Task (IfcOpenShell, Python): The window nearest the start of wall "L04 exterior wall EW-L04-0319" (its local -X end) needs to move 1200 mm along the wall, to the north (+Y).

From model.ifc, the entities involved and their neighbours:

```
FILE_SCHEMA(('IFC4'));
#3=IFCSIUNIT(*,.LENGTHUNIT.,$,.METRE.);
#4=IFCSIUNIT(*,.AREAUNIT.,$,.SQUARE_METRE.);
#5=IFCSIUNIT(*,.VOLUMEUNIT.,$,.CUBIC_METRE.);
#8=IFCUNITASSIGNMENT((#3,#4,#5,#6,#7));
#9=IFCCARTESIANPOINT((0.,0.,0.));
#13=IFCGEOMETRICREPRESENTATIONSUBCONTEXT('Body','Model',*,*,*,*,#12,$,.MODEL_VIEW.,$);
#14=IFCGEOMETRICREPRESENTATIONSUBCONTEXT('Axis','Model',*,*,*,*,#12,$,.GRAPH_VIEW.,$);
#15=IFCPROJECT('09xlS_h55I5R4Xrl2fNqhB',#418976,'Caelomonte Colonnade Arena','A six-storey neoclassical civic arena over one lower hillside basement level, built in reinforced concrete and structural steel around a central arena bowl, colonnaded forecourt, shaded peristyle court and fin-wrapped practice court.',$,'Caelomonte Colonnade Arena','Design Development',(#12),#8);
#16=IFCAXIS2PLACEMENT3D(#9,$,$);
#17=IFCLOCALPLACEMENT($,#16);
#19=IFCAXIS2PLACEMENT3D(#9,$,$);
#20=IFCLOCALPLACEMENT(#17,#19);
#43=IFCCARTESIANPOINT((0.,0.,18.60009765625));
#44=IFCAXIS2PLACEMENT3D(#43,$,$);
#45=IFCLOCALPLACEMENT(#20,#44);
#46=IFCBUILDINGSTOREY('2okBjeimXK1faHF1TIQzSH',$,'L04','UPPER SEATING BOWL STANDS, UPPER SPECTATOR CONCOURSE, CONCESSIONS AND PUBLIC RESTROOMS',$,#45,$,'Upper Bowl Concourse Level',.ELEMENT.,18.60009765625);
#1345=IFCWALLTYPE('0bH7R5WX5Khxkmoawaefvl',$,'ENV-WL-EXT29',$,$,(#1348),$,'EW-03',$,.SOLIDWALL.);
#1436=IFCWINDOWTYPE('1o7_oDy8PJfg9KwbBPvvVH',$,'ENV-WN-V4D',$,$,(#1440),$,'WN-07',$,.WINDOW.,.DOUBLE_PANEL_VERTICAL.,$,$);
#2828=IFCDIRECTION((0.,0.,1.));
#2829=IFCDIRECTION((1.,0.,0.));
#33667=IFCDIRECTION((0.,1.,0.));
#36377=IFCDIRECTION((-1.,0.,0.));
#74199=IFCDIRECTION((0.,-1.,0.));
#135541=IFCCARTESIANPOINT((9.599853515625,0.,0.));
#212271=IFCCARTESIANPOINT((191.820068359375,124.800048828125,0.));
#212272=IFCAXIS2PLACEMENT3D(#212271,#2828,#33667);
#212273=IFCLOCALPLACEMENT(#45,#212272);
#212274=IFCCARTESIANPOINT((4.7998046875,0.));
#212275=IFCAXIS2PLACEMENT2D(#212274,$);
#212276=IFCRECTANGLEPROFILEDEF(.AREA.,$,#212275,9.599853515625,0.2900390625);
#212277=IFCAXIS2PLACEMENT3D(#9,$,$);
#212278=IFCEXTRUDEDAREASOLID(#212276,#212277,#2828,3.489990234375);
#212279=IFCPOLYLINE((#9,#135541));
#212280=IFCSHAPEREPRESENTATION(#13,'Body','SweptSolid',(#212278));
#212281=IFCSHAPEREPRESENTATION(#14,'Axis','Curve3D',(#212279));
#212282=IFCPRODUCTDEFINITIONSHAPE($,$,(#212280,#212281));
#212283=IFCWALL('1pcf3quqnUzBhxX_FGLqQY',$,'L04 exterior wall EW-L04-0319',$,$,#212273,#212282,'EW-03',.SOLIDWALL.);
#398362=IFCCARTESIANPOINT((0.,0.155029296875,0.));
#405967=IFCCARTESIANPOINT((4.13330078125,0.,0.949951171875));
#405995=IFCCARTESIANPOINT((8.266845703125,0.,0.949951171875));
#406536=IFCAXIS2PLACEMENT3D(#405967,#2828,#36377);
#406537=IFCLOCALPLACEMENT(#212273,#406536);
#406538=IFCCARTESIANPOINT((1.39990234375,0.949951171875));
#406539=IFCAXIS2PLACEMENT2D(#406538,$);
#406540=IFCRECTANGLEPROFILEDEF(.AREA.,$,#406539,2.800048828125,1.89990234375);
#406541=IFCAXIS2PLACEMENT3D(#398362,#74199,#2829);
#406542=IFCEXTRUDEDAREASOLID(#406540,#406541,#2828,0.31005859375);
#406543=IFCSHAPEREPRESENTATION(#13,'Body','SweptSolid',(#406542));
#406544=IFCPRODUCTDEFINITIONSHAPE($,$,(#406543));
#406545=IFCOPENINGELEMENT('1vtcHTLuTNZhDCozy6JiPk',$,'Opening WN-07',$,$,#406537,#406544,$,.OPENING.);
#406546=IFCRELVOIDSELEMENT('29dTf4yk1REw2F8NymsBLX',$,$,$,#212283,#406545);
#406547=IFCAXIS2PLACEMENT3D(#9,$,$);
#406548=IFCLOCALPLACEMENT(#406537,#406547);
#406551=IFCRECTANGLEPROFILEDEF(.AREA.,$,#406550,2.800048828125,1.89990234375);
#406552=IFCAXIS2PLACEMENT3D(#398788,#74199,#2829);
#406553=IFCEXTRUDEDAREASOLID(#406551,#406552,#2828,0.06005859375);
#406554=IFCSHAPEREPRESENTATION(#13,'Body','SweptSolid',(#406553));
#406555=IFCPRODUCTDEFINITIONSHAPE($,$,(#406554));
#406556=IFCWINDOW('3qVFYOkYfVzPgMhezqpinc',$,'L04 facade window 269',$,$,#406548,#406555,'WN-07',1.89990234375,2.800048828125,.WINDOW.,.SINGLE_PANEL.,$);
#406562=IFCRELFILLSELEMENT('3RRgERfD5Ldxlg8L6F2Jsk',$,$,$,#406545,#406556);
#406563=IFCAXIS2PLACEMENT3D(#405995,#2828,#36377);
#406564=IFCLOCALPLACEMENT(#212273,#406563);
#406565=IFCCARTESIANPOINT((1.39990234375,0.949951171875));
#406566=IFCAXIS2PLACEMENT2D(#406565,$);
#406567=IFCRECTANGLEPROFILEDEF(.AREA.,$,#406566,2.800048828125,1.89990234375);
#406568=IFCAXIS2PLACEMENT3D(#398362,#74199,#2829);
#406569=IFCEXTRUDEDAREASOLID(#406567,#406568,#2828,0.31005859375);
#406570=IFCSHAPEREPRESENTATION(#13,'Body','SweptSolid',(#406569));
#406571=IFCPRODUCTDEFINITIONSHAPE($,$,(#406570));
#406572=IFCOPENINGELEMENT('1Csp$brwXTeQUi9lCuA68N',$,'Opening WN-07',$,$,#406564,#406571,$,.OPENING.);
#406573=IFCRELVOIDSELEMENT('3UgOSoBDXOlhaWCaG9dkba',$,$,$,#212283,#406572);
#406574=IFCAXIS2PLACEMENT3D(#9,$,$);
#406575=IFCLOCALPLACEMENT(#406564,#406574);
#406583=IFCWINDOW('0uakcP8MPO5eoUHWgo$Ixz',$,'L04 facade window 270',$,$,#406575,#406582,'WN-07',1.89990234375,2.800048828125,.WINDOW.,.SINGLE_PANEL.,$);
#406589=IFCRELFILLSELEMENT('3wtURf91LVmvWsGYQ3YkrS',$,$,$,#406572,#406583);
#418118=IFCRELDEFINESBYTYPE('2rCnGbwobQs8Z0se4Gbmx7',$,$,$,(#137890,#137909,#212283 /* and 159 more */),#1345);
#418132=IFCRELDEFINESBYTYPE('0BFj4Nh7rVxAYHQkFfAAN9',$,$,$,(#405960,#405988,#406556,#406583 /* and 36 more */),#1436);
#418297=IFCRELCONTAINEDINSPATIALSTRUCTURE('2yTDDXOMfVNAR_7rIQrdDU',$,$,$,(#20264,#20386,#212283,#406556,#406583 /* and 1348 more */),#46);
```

```python
import ifcopenshell
import ifcopenshell.api.geometry
import ifcopenshell.util.placement
import ifcopenshell.util.unit

model = ifcopenshell.open("model.ifc")
unit_scale = ifcopenshell.util.unit.calculate_unit_scale(model)

window = model.by_guid("3qVFYOkYfVzPgMhezqpinc")
opening = window.FillsVoids[0].RelatingOpeningElement
wall = opening.VoidsElements[0].RelatingBuildingElement

wall_matrix = ifcopenshell.util.placement.get_local_placement(wall.ObjectPlacement)
shift = wall_matrix[:3, 0] * 1.2 / unit_scale
before = ifcopenshell.util.placement.get_local_placement(window.ObjectPlacement)[:3, 3].copy()

# The window is placed relative to its opening, so it follows when the opening moves.
matrix = ifcopenshell.util.placement.get_local_placement(opening.ObjectPlacement)
matrix[:3, 3] += shift
ifcopenshell.api.geometry.edit_object_placement(
    model, product=opening, matrix=matrix, is_si=False, should_transform_children=True
)

after = ifcopenshell.util.placement.get_local_placement(window.ObjectPlacement)[:3, 3]
print("window moved by", (after - before).round(3) + 0.0)

model.write("model_updated.ifc")
```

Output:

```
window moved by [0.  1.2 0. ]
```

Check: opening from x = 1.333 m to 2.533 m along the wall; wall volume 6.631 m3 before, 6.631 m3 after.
